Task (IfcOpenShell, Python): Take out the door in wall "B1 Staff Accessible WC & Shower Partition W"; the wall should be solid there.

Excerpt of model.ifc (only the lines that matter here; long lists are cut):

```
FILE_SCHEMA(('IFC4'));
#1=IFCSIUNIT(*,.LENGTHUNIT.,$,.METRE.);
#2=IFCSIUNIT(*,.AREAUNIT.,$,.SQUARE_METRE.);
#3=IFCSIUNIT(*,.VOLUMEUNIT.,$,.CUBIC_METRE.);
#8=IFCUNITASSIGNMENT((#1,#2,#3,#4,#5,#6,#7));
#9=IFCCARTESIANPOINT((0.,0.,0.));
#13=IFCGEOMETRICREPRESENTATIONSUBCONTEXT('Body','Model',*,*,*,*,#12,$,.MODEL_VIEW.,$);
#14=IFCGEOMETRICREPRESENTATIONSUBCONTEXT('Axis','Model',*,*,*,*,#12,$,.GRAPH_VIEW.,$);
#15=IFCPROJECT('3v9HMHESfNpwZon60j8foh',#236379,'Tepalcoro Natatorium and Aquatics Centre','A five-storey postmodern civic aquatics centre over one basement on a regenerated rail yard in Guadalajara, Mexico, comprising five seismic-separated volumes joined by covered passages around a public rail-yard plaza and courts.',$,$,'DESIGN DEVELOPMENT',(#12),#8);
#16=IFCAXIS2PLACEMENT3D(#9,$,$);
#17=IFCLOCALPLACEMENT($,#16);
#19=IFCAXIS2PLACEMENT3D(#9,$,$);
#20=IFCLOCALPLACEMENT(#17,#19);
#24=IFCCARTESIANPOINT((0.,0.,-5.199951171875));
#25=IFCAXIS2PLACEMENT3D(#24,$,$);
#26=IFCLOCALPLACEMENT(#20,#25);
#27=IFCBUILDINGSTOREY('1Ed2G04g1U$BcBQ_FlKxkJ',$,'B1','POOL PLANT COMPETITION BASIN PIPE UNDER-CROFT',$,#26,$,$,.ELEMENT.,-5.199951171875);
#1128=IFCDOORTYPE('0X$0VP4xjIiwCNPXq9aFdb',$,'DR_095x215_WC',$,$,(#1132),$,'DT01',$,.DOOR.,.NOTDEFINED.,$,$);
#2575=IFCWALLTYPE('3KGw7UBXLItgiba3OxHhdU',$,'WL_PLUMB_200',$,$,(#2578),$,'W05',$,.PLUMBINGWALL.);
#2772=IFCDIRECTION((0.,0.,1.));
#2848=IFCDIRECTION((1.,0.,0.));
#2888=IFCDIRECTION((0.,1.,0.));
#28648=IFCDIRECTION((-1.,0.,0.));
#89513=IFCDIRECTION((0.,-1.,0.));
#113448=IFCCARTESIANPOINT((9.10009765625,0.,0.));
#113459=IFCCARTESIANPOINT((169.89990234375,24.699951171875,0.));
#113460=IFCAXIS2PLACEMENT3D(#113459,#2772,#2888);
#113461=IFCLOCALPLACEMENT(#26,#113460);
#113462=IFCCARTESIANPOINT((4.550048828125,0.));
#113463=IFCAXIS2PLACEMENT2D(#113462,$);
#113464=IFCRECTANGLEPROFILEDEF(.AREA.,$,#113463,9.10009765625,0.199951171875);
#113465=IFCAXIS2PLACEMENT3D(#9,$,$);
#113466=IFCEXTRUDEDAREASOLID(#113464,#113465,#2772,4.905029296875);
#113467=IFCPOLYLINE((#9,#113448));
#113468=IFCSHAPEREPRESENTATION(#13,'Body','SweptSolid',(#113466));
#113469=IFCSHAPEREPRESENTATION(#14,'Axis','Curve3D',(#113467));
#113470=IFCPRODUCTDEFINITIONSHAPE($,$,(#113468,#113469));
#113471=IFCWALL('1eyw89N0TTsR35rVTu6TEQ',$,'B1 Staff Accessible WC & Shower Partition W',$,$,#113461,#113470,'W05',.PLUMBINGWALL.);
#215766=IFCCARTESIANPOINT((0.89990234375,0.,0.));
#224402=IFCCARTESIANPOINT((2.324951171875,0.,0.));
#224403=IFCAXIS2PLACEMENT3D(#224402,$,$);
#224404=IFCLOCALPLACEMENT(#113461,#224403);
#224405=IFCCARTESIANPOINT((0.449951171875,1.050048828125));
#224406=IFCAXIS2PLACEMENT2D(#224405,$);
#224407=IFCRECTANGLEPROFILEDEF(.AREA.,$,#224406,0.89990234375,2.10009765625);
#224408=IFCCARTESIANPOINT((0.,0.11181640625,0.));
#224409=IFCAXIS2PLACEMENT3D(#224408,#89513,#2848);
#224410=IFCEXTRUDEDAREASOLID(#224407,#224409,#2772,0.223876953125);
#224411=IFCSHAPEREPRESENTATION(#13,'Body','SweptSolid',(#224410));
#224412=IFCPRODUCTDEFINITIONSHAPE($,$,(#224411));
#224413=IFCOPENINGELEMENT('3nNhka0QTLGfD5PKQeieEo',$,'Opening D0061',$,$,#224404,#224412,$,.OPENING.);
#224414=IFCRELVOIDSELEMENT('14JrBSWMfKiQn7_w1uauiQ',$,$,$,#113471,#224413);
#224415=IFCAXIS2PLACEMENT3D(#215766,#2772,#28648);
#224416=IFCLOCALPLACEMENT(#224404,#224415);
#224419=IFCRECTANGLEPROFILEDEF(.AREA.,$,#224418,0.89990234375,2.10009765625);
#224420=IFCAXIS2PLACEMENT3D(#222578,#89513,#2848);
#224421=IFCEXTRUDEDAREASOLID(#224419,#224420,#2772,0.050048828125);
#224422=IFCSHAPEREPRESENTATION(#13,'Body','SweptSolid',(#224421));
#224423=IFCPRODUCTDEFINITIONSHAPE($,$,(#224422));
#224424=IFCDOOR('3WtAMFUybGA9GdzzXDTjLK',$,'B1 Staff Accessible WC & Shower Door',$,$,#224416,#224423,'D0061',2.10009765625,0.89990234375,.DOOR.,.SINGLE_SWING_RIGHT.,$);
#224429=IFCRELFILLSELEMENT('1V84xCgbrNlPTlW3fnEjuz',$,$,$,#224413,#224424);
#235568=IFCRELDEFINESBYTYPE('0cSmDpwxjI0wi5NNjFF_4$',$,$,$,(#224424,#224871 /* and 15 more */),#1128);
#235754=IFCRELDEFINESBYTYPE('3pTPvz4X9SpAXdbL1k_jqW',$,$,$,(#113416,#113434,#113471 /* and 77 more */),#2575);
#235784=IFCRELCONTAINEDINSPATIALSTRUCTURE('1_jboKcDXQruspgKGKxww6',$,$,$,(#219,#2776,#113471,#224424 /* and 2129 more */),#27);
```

```python
import ifcopenshell
import ifcopenshell.api.feature
import ifcopenshell.api.root
import ifcopenshell.geom
import ifcopenshell.util.shape

model = ifcopenshell.open("model.ifc")
settings = ifcopenshell.geom.settings()


def volume(element):
    """Net volume in cubic metres, openings subtracted."""
    shape = ifcopenshell.geom.create_shape(settings, element)
    return ifcopenshell.util.shape.get_volume(shape.geometry)


door = model.by_id(224424)
opening = door.FillsVoids[0].RelatingOpeningElement
wall = opening.VoidsElements[0].RelatingBuildingElement
before = volume(wall)

ifcopenshell.api.root.remove_product(model, product=door)
ifcopenshell.api.feature.remove_feature(model, feature=opening)

after = volume(wall)

print(f"wall volume {before:.3f} -> {after:.3f} m3")

model.write("model_v2.ifc")
```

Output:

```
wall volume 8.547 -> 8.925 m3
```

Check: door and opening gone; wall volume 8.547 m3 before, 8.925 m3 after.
